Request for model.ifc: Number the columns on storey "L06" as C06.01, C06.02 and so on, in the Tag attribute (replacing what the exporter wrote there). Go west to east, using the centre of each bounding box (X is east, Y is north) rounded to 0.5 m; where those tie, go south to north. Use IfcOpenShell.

First a look at what the model holds.

```python
import ifcopenshell
import ifcopenshell.util.element
import ifcopenshell.util.placement

model = ifcopenshell.open("model.ifc")
print(model.schema)
storey = next(s for s in model.by_type("IfcBuildingStorey") if s.Name == "L06")
columns = [e for e in ifcopenshell.util.element.get_decomposition(storey) if e.is_a("IfcColumn")]
for e in sorted(columns, key=lambda e: e.id()):
    origin = ifcopenshell.util.placement.get_local_placement(e.ObjectPlacement)[:3, 3]
    print(e.id(), e.Tag, e.Name, origin.round(2) + 0.0, sep=" | ")
```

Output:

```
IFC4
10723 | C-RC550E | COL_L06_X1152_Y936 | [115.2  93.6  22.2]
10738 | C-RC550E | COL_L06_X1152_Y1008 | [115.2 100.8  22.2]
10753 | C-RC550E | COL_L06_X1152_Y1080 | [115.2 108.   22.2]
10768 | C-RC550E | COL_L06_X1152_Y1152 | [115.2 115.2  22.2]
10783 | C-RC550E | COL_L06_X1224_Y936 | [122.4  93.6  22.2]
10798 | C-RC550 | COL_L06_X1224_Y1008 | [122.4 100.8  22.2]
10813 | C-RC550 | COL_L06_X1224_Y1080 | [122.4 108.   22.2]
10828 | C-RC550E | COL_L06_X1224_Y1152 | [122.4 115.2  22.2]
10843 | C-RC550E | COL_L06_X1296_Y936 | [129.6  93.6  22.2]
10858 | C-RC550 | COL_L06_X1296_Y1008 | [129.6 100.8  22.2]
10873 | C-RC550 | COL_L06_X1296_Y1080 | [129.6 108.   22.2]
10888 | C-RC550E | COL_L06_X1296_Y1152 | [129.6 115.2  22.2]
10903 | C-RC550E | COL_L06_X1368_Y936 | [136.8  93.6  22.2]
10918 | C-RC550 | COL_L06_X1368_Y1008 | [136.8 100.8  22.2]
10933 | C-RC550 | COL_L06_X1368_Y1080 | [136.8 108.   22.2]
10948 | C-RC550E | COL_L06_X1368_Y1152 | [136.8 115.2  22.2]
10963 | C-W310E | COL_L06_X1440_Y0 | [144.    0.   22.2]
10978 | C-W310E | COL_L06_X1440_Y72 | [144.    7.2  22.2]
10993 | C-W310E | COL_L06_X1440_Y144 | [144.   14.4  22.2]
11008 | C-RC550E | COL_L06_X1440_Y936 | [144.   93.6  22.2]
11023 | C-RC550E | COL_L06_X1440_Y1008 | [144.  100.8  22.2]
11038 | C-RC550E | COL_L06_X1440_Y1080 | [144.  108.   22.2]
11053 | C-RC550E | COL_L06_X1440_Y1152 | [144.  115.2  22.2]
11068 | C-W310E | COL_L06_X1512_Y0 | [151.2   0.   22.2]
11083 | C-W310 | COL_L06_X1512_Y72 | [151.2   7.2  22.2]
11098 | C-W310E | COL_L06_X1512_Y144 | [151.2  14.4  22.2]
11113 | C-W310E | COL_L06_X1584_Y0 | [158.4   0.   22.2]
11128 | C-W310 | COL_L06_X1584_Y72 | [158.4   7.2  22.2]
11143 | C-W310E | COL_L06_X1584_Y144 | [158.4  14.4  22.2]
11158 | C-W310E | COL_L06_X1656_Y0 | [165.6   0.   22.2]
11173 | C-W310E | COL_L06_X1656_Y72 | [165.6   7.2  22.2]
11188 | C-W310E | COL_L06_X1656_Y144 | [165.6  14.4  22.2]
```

```python
import ifcopenshell
import ifcopenshell.geom
import ifcopenshell.util.element
import ifcopenshell.util.shape

model = ifcopenshell.open("model.ifc")
settings = ifcopenshell.geom.settings()
settings.set("use-world-coords", True)


def centre(element):
    shape = ifcopenshell.geom.create_shape(settings, element)
    return ifcopenshell.util.shape.get_bbox_centroid(shape.geometry)


storey = next(s for s in model.by_type("IfcBuildingStorey") if s.Name == "L06")
columns = [e for e in ifcopenshell.util.element.get_decomposition(storey) if e.is_a("IfcColumn")]

# Insertion points can sit at a corner or the storey origin, so sort by the geometry (in metres).
centres = {e: centre(e) for e in columns}
columns.sort(key=lambda e: (round(centres[e][0] / 0.5), centres[e][1]))

for i, e in enumerate(columns, start=1):
    number = f"C06.{i:02d}"
    e.Tag = number
    print(e.id(), number)

model.write("model_edited.ifc")
```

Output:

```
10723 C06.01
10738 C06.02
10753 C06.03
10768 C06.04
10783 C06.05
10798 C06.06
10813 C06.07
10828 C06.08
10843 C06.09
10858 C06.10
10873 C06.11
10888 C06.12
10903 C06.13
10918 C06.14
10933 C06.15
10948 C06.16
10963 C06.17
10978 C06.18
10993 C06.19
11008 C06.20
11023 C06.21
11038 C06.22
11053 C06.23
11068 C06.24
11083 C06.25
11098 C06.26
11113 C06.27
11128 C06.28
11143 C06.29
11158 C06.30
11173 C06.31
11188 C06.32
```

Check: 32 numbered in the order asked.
